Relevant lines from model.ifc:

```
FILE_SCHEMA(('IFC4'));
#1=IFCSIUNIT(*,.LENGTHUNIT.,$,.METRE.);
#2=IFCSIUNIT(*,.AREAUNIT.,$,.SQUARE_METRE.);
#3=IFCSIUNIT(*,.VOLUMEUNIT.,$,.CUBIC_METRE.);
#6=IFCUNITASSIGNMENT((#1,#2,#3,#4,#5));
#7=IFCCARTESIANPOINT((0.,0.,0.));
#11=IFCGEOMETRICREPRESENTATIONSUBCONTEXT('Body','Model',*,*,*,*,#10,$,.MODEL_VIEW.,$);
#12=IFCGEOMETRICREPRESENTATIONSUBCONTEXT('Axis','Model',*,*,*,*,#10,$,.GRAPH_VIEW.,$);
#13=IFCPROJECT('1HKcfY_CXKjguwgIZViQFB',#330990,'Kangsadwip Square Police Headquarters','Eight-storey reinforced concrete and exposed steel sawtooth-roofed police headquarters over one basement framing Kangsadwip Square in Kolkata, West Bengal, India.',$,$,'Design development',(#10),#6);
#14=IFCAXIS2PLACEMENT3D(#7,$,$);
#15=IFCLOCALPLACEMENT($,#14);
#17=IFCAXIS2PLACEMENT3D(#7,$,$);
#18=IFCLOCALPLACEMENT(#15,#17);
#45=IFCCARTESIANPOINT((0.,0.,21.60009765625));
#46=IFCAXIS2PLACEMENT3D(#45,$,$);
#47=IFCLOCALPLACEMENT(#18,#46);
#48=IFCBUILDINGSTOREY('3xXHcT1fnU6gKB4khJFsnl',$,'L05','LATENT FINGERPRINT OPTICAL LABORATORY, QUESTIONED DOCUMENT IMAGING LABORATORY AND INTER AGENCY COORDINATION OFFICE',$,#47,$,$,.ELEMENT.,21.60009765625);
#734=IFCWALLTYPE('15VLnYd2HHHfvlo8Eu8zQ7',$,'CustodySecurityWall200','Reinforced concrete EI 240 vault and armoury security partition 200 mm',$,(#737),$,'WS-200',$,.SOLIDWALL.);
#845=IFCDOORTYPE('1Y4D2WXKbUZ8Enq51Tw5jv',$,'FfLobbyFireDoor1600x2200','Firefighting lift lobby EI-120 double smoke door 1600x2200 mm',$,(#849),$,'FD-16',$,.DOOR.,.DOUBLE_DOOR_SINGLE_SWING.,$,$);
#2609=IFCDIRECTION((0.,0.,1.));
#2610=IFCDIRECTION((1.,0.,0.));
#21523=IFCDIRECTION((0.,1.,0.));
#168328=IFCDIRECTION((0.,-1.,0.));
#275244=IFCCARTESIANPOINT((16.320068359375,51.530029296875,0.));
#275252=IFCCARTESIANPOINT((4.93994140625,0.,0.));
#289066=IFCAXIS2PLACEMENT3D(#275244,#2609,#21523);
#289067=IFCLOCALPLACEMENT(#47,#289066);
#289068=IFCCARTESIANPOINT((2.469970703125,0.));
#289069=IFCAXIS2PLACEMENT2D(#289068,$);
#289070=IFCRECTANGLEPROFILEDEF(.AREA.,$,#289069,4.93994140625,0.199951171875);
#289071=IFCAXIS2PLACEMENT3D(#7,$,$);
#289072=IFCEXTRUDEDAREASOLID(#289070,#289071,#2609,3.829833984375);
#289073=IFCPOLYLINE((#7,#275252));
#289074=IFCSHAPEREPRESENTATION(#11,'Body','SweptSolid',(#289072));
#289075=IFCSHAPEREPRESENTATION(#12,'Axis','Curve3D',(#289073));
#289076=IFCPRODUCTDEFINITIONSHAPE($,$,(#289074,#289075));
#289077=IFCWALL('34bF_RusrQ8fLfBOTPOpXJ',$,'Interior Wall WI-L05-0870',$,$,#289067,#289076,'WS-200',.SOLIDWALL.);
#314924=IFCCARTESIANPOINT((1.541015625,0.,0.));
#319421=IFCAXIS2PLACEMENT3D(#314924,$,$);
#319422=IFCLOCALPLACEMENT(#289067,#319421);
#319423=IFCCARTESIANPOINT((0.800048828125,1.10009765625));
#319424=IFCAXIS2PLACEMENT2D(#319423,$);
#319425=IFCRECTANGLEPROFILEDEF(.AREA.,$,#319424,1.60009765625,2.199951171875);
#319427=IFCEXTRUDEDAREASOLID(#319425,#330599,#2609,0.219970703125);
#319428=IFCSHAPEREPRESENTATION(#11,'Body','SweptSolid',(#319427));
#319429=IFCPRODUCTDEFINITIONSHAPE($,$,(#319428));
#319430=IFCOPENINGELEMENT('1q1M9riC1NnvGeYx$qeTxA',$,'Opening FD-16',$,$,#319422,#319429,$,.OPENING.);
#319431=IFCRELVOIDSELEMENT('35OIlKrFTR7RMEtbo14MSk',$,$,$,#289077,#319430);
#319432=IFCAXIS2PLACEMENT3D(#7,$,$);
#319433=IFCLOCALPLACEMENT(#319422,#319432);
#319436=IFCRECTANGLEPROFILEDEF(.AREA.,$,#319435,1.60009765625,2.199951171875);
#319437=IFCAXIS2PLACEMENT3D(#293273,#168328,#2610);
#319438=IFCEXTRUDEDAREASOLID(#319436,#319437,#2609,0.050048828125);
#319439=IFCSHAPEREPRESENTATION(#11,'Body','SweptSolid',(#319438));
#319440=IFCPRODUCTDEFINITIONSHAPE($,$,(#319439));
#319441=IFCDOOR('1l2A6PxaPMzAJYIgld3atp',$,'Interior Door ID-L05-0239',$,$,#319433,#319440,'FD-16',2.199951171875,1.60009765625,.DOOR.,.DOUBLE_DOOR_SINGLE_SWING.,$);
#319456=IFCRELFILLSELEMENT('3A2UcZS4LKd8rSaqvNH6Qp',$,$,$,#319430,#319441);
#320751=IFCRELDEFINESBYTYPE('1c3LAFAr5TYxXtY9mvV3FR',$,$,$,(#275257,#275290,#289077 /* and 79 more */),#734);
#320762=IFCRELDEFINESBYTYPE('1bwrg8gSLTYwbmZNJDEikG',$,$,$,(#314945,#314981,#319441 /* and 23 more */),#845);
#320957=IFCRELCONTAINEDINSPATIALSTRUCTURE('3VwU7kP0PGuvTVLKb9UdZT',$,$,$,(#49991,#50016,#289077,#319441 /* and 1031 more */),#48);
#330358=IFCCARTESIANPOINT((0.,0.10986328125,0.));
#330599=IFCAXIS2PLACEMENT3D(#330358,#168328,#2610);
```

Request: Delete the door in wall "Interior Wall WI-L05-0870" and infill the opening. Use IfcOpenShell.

```python
import ifcopenshell
import ifcopenshell.api.feature
import ifcopenshell.api.root
import ifcopenshell.geom
import ifcopenshell.util.shape

model = ifcopenshell.open("model.ifc")
settings = ifcopenshell.geom.settings()


def volume(element):
    """Net volume in cubic metres, openings subtracted."""
    shape = ifcopenshell.geom.create_shape(settings, element)
    return ifcopenshell.util.shape.get_volume(shape.geometry)


door = model.by_id(319441)
opening = door.FillsVoids[0].RelatingOpeningElement
wall = opening.VoidsElements[0].RelatingBuildingElement
before = volume(wall)

ifcopenshell.api.root.remove_product(model, product=door)
ifcopenshell.api.feature.remove_feature(model, feature=opening)

after = volume(wall)

print(f"wall volume {before:.3f} -> {after:.3f} m3")

model.write("model_edited.ifc")
```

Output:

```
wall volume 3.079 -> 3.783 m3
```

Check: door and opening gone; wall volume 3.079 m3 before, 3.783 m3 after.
